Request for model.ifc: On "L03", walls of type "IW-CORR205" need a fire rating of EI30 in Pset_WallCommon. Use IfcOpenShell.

First a look at what the model holds.

```python
import ifcopenshell
import ifcopenshell.util.element

model = ifcopenshell.open("model.ifc")
print(model.schema)
storey = next(s for s in model.by_type("IfcBuildingStorey") if s.Name == "L03")
walls = [e for e in ifcopenshell.util.element.get_decomposition(storey) if e.is_a("IfcWall")]
seen = {}
for e in walls:
    element_type = ifcopenshell.util.element.get_type(e)
    key = (element_type.Name if element_type != e and element_type else None, ifcopenshell.util.element.get_pset(e, "Pset_WallCommon", "FireRating"))
    seen[key] = seen.get(key, 0) + 1
for (name, value), count in sorted(seen.items(), key=str):
    print(count, "x", name, "|", value)
```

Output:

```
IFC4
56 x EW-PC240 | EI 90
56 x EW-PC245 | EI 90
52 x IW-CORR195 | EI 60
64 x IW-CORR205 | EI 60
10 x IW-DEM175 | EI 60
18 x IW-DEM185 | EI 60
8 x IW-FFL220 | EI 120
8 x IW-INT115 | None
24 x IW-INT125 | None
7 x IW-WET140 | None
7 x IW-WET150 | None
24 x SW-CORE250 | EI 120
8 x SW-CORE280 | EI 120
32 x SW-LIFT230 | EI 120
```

```python
import ifcopenshell
import ifcopenshell.api.pset
import ifcopenshell.util.element

model = ifcopenshell.open("model.ifc")

storey = next(s for s in model.by_type("IfcBuildingStorey") if s.Name == "L03")
walls = [e for e in ifcopenshell.util.element.get_decomposition(storey) if e.is_a("IfcWall")]

count = 0
for e in walls:
    element_type = ifcopenshell.util.element.get_type(e)
    if element_type in (None, e) or element_type.Name != "IW-CORR205":
        continue
    # add_pset returns the element's existing set when there is one.
    pset = ifcopenshell.api.pset.add_pset(model, product=e, name="Pset_WallCommon")
    ifcopenshell.api.pset.edit_pset(model, pset=pset, properties={"FireRating": "EI30"})
    count += 1

print(count, "walls updated")

model.write("model-out.ifc")
```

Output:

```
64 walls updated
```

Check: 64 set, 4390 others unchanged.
